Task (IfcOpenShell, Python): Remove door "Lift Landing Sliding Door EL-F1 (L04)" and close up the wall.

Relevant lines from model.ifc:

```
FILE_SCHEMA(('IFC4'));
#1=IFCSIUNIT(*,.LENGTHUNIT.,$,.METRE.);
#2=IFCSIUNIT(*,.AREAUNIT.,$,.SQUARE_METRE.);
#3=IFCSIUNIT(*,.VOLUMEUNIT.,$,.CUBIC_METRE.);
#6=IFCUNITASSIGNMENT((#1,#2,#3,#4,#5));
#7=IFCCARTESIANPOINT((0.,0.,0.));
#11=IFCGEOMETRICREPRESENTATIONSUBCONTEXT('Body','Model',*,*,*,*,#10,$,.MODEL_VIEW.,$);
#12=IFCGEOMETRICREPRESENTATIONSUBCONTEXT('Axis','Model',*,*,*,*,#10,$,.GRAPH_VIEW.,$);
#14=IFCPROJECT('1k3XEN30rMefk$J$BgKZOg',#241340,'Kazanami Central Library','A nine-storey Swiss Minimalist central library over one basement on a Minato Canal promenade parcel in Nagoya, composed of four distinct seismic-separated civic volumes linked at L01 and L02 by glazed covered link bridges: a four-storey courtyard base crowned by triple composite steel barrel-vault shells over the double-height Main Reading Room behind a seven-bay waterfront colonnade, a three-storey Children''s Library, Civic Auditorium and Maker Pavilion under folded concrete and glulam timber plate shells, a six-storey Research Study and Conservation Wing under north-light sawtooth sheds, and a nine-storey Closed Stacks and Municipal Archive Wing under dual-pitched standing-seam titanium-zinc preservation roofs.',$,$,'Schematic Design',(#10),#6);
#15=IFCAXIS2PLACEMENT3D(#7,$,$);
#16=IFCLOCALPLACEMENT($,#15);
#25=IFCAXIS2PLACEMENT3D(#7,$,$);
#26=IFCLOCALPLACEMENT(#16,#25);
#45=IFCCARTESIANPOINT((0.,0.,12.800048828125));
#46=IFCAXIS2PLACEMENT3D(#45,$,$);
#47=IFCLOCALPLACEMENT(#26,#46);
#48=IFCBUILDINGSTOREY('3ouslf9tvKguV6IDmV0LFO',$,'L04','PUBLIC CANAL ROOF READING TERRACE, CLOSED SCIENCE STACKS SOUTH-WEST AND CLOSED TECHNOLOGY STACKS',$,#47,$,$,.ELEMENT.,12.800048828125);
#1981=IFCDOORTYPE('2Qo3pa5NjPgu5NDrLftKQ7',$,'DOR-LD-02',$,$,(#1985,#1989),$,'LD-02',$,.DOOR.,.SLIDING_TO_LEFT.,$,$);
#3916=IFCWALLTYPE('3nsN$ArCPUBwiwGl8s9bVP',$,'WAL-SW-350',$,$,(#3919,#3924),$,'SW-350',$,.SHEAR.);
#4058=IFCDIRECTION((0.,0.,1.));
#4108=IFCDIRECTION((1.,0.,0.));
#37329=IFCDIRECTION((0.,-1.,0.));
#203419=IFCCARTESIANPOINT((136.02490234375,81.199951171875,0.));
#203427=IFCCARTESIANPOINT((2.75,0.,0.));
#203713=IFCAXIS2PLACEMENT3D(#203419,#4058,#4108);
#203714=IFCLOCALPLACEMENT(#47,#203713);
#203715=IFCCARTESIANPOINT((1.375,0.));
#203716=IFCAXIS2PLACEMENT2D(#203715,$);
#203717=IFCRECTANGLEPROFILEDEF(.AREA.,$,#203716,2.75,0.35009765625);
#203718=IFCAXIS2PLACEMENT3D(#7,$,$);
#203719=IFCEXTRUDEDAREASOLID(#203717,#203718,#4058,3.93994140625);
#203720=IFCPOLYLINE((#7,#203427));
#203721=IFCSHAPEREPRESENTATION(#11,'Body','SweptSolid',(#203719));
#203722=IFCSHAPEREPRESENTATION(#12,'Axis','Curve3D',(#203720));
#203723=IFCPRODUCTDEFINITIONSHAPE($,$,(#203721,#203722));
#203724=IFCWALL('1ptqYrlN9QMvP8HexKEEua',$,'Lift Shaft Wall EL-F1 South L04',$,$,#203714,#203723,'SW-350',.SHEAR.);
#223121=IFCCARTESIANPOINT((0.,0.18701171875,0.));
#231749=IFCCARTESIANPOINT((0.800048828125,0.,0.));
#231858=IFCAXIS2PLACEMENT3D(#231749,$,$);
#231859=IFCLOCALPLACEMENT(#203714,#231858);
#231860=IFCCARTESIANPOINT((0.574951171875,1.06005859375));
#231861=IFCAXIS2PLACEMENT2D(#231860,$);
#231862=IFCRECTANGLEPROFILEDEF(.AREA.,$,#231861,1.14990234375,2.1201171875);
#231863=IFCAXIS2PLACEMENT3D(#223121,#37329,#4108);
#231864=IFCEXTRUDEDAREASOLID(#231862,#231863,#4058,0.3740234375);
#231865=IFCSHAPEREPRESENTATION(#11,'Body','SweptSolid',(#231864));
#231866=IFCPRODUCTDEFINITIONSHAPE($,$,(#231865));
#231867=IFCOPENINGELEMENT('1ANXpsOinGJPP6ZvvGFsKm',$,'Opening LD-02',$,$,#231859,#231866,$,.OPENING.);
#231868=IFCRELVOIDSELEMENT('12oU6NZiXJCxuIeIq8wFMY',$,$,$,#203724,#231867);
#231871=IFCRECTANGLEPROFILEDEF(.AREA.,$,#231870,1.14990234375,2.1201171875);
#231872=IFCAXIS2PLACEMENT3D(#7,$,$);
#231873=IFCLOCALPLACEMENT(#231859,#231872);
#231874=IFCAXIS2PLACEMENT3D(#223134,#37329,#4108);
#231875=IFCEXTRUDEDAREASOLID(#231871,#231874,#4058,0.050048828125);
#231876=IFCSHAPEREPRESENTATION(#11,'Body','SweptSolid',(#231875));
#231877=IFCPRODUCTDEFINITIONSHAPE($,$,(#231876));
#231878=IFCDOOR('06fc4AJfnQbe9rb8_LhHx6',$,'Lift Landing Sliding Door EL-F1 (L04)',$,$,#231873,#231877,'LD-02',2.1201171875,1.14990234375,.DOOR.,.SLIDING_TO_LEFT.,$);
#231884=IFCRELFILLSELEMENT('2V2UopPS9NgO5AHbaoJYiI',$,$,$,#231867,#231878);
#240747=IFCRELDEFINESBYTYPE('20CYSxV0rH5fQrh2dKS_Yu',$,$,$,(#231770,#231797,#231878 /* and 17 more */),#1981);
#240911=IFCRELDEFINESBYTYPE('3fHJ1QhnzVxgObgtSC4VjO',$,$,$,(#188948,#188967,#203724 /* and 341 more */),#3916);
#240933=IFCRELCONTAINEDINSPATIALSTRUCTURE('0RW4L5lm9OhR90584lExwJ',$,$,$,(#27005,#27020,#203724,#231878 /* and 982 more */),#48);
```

```python
import ifcopenshell
import ifcopenshell.api.feature
import ifcopenshell.api.root
import ifcopenshell.geom
import ifcopenshell.util.shape

model = ifcopenshell.open("model.ifc")
settings = ifcopenshell.geom.settings()


def volume(element):
    """Net volume in cubic metres, openings subtracted."""
    shape = ifcopenshell.geom.create_shape(settings, element)
    return ifcopenshell.util.shape.get_volume(shape.geometry)


door = model.by_guid("06fc4AJfnQbe9rb8_LhHx6")
opening = door.FillsVoids[0].RelatingOpeningElement
wall = opening.VoidsElements[0].RelatingBuildingElement
before = volume(wall)

ifcopenshell.api.root.remove_product(model, product=door)
ifcopenshell.api.feature.remove_feature(model, feature=opening)

after = volume(wall)

print(f"wall volume {before:.3f} -> {after:.3f} m3")

model.write("model-out.ifc")
```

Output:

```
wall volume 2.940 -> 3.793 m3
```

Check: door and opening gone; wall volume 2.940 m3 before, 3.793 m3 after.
